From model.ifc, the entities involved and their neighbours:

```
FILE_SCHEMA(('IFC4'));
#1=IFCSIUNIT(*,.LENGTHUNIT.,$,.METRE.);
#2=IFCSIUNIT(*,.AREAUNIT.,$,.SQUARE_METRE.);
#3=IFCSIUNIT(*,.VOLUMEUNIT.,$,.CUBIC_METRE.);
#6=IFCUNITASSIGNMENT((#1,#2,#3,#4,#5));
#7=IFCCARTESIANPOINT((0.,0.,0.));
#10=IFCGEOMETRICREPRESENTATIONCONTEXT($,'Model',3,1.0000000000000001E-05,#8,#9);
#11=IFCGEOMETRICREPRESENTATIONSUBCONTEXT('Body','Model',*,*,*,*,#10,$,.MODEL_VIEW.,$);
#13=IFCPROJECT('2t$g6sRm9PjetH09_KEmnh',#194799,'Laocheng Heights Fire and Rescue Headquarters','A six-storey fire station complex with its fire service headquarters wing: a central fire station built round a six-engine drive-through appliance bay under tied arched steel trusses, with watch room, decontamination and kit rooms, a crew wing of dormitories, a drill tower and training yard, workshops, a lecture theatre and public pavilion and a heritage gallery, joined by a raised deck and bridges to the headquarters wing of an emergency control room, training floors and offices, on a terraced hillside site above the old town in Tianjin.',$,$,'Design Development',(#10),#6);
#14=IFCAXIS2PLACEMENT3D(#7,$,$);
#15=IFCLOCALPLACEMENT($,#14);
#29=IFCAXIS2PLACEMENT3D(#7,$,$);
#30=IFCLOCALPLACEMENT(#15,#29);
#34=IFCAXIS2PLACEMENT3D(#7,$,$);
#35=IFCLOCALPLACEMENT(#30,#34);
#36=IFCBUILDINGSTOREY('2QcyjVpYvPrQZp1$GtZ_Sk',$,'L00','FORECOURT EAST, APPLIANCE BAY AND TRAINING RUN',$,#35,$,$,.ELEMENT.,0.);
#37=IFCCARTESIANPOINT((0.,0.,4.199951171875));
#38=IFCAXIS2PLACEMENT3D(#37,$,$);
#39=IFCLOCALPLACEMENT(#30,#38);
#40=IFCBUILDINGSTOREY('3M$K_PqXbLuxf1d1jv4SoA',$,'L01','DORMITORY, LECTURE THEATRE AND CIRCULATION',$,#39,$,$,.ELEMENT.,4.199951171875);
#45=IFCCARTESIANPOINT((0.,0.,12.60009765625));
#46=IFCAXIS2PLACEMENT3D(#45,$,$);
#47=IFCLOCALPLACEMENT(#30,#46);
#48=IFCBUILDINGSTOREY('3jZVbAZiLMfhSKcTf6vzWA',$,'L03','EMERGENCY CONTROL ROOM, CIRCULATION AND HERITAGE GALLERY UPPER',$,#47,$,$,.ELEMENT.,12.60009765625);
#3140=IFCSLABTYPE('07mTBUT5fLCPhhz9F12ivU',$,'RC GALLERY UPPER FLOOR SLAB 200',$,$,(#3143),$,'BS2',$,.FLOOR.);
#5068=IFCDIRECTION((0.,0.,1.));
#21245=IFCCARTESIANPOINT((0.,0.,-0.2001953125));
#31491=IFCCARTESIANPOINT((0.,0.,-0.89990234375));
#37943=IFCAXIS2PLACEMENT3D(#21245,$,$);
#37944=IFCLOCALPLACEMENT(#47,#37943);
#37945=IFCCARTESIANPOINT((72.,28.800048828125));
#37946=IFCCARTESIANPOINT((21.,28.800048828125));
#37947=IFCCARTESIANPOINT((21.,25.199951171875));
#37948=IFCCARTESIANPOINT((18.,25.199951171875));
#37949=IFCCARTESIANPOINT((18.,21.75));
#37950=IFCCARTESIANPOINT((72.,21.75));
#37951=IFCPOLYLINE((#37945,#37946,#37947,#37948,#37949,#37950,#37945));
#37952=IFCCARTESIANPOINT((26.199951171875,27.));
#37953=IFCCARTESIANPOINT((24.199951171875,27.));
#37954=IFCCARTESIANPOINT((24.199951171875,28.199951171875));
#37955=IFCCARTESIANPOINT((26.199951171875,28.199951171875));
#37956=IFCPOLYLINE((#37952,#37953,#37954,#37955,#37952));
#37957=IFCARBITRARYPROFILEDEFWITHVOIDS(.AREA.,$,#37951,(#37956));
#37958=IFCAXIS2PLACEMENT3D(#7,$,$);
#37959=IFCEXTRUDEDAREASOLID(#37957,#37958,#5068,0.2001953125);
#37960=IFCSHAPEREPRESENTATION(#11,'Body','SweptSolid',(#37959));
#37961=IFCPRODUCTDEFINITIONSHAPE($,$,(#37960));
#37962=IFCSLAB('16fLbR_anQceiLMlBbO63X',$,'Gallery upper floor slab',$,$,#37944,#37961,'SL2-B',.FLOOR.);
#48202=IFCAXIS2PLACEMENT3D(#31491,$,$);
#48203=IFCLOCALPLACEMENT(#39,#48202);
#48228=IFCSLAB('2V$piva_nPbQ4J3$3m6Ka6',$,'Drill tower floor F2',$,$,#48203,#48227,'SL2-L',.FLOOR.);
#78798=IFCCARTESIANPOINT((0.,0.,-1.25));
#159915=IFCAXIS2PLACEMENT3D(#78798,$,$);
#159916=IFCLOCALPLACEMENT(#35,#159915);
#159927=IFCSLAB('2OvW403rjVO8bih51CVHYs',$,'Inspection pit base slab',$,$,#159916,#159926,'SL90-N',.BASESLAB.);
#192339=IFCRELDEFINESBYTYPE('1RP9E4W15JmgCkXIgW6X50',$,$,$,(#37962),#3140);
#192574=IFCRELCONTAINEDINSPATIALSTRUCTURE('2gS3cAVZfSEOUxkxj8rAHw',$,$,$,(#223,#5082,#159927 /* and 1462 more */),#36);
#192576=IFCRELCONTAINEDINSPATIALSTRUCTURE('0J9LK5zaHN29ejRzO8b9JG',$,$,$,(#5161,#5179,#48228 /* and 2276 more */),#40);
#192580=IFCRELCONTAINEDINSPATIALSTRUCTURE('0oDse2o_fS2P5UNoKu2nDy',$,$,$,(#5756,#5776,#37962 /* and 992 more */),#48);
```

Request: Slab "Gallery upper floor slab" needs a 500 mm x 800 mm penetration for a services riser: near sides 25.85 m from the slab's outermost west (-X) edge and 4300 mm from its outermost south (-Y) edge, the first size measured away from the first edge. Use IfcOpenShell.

```python
import numpy as np
import ifcopenshell
import ifcopenshell.api.feature
import ifcopenshell.api.geometry
import ifcopenshell.api.root
import ifcopenshell.geom
import ifcopenshell.util.placement
import ifcopenshell.util.representation
import ifcopenshell.util.shape
import ifcopenshell.util.unit

model = ifcopenshell.open("model.ifc")
unit_scale = ifcopenshell.util.unit.calculate_unit_scale(model)
settings = ifcopenshell.geom.settings()


def volume(element):
    """Net volume in cubic metres, openings subtracted."""
    shape = ifcopenshell.geom.create_shape(settings, element)
    return ifcopenshell.util.shape.get_volume(shape.geometry)


slab = model.by_guid("16fLbR_anQceiLMlBbO63X")
before = volume(slab)

# Extent in the slab's own axes, in metres. The edges named are its -X and -Y sides.
slab_shape = ifcopenshell.geom.create_shape(settings, slab)
vertices = ifcopenshell.util.shape.get_vertices(slab_shape.geometry)
x_min, y_min, bottom = vertices.min(axis=0)
top = vertices[:, 2].max()

opening = ifcopenshell.api.root.create_entity(model, ifc_class="IfcOpeningElement", name="Services riser opening", predefined_type="OPENING")
context = ifcopenshell.util.representation.get_context(model, "Model", "Body", "MODEL_VIEW")
width, depth = 0.5, 0.8
outline = [(0.0, 0.0), (width, 0.0), (width, depth), (0.0, depth), (0.0, 0.0)]
# Overshoot both faces by 50 mm so the cut is clean.
shape = ifcopenshell.api.geometry.add_slab_representation(
    model, context=context, depth=top - bottom + 0.1, polyline=outline
)
ifcopenshell.api.geometry.assign_representation(model, product=opening, representation=shape)

matrix = ifcopenshell.util.placement.get_local_placement(slab.ObjectPlacement)
matrix[:, 3] = matrix @ np.append(np.array([x_min + 25.85, y_min + 4.3, bottom - 0.05]) / unit_scale, 1.0)
ifcopenshell.api.geometry.edit_object_placement(model, product=opening, matrix=matrix, is_si=False)
ifcopenshell.api.feature.add_feature(model, feature=opening, element=slab)

after = volume(slab)

print(f"slab volume {before:.3f} -> {after:.3f} m3")

model.write("model_updated.ifc")
```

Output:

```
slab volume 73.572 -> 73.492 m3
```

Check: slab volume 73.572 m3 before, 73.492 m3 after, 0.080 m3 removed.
